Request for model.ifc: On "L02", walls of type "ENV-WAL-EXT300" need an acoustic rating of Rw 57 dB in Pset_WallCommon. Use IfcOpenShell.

First a look at what the model holds.

```python
import ifcopenshell
import ifcopenshell.util.element

model = ifcopenshell.open("model.ifc")
print(model.schema)
storey = next(s for s in model.by_type("IfcBuildingStorey") if s.Name == "L02")
walls = [e for e in ifcopenshell.util.element.get_decomposition(storey) if e.is_a("IfcWall")]
seen = {}
for e in walls:
    element_type = ifcopenshell.util.element.get_type(e)
    key = (element_type.Name if element_type != e and element_type else None, ifcopenshell.util.element.get_pset(e, "Pset_WallCommon", "AcousticRating"))
    seen[key] = seen.get(key, 0) + 1
for (name, value), count in sorted(seen.items(), key=str):
    print(count, "x", name, "|", value)
```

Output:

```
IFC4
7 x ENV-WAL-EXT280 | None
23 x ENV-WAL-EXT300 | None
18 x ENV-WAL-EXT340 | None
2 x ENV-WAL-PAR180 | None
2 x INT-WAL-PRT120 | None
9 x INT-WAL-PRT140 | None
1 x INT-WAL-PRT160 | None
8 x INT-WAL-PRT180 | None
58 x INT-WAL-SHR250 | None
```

```python
import ifcopenshell
import ifcopenshell.api.pset
import ifcopenshell.util.element

model = ifcopenshell.open("model.ifc")

storey = next(s for s in model.by_type("IfcBuildingStorey") if s.Name == "L02")
walls = [e for e in ifcopenshell.util.element.get_decomposition(storey) if e.is_a("IfcWall")]

count = 0
for e in walls:
    element_type = ifcopenshell.util.element.get_type(e)
    if element_type in (None, e) or element_type.Name != "ENV-WAL-EXT300":
        continue
    # add_pset returns the element's existing set when there is one.
    pset = ifcopenshell.api.pset.add_pset(model, product=e, name="Pset_WallCommon")
    ifcopenshell.api.pset.edit_pset(model, pset=pset, properties={"AcousticRating": "Rw 57 dB"})
    count += 1

print(count, "walls updated")

model.write("model_updated.ifc")
```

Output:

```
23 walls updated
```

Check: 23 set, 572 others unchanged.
